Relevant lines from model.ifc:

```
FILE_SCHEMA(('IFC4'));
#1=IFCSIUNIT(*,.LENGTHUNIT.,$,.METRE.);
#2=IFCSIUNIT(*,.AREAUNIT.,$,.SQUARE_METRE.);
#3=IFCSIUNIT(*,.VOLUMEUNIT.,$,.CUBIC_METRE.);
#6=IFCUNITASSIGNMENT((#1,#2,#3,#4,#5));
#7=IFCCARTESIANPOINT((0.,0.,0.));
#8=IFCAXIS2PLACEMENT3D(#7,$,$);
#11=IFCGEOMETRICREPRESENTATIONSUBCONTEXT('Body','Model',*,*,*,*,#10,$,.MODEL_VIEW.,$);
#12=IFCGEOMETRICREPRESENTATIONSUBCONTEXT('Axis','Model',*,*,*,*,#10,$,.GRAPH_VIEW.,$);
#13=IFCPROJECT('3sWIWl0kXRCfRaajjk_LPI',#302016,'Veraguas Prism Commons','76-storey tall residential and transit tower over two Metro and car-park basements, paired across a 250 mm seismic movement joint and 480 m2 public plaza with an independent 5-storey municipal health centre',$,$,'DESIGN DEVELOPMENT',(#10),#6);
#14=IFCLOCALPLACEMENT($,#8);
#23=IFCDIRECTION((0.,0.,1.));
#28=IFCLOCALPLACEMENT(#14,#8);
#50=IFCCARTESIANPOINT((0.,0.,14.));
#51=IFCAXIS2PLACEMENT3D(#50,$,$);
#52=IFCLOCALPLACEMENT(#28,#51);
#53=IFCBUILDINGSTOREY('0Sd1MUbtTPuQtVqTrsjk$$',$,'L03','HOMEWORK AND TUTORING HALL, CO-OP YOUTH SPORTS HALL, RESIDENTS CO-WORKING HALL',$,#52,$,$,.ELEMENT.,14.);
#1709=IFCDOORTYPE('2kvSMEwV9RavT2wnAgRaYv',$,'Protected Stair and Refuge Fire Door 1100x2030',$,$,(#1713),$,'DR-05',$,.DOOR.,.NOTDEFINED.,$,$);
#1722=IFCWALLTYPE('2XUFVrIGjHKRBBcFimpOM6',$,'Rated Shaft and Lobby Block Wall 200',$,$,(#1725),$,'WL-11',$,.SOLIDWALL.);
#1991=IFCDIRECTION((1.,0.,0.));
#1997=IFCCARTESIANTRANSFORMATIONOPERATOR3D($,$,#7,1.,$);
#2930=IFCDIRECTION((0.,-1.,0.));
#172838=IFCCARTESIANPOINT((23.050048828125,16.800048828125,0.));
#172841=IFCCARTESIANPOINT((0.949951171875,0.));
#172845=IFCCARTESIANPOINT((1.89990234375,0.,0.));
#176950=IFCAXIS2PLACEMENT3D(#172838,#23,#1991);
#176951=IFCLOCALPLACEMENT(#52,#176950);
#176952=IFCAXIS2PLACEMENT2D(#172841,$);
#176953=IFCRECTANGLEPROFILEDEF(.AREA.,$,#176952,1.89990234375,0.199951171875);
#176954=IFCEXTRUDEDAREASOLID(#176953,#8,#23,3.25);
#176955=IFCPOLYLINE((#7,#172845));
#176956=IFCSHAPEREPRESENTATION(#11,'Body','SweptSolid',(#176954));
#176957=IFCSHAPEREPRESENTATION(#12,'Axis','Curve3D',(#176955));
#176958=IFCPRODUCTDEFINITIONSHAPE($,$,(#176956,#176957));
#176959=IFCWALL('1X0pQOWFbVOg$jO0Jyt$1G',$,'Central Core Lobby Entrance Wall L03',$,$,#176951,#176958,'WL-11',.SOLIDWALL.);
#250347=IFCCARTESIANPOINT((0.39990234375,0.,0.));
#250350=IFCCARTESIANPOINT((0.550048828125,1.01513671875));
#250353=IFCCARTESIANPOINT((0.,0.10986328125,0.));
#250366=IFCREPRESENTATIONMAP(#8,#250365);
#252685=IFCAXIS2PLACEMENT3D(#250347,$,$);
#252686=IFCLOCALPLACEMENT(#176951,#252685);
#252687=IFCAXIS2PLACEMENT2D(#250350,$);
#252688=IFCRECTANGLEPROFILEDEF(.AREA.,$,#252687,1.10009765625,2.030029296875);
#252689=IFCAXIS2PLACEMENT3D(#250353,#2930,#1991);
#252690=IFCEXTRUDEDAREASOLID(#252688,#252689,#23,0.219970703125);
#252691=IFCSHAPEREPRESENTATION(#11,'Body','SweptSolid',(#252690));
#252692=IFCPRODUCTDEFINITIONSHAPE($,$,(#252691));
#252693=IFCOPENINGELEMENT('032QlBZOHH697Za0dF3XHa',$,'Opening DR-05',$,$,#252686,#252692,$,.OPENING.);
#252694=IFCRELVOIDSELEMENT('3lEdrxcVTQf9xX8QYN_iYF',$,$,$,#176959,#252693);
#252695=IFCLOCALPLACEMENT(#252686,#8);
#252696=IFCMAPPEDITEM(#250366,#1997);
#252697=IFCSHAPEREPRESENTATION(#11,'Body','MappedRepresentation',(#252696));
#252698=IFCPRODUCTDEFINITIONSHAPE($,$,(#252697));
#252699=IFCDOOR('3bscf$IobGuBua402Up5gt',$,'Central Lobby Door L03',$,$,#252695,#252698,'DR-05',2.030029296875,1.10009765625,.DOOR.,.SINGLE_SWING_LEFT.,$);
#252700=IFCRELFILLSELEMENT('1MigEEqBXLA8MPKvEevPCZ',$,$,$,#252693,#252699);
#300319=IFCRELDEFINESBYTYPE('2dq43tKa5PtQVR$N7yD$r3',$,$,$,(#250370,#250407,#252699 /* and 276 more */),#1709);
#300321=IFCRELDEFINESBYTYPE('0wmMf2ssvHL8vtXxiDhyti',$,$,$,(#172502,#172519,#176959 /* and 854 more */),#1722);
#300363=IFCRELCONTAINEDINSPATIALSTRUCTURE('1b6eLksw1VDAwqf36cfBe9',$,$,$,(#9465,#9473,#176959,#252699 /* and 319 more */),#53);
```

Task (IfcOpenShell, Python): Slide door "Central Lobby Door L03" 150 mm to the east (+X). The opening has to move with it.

```python
import ifcopenshell
import ifcopenshell.api.geometry
import ifcopenshell.util.placement
import ifcopenshell.util.unit

model = ifcopenshell.open("model.ifc")
unit_scale = ifcopenshell.util.unit.calculate_unit_scale(model)

door = model.by_guid("3bscf$IobGuBua402Up5gt")
opening = door.FillsVoids[0].RelatingOpeningElement
wall = opening.VoidsElements[0].RelatingBuildingElement

wall_matrix = ifcopenshell.util.placement.get_local_placement(wall.ObjectPlacement)
shift = wall_matrix[:3, 0] * 0.15 / unit_scale
before = ifcopenshell.util.placement.get_local_placement(door.ObjectPlacement)[:3, 3].copy()

# The door is placed relative to its opening, so it follows when the opening moves.
matrix = ifcopenshell.util.placement.get_local_placement(opening.ObjectPlacement)
matrix[:3, 3] += shift
ifcopenshell.api.geometry.edit_object_placement(
    model, product=opening, matrix=matrix, is_si=False, should_transform_children=True
)

after = ifcopenshell.util.placement.get_local_placement(door.ObjectPlacement)[:3, 3]
print("door moved by", (after - before).round(3) + 0.0)

model.write("model_rev.ifc")
```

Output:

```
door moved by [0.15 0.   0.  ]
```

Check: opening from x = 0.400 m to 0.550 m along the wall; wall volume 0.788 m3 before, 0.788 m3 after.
